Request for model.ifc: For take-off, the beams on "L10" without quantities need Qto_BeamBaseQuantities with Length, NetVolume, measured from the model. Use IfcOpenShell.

First a look at what the model holds.

```python
import ifcopenshell
import ifcopenshell.util.element
import ifcopenshell.util.unit

model = ifcopenshell.open("model.ifc")
print(model.schema)
for unit_type in ("LENGTHUNIT", "AREAUNIT", "VOLUMEUNIT"):
    print(unit_type, ifcopenshell.util.unit.calculate_unit_scale(model, unit_type))
storey = next(s for s in model.by_type("IfcBuildingStorey") if s.Name == "L10")
beams = [e for e in ifcopenshell.util.element.get_decomposition(storey) if e.is_a("IfcBeam")]
for e in sorted(beams, key=lambda e: e.id()):
    print(e.id(), e.is_a(), e.Name, list(ifcopenshell.util.element.get_psets(e, qtos_only=True)), sep=" | ")
```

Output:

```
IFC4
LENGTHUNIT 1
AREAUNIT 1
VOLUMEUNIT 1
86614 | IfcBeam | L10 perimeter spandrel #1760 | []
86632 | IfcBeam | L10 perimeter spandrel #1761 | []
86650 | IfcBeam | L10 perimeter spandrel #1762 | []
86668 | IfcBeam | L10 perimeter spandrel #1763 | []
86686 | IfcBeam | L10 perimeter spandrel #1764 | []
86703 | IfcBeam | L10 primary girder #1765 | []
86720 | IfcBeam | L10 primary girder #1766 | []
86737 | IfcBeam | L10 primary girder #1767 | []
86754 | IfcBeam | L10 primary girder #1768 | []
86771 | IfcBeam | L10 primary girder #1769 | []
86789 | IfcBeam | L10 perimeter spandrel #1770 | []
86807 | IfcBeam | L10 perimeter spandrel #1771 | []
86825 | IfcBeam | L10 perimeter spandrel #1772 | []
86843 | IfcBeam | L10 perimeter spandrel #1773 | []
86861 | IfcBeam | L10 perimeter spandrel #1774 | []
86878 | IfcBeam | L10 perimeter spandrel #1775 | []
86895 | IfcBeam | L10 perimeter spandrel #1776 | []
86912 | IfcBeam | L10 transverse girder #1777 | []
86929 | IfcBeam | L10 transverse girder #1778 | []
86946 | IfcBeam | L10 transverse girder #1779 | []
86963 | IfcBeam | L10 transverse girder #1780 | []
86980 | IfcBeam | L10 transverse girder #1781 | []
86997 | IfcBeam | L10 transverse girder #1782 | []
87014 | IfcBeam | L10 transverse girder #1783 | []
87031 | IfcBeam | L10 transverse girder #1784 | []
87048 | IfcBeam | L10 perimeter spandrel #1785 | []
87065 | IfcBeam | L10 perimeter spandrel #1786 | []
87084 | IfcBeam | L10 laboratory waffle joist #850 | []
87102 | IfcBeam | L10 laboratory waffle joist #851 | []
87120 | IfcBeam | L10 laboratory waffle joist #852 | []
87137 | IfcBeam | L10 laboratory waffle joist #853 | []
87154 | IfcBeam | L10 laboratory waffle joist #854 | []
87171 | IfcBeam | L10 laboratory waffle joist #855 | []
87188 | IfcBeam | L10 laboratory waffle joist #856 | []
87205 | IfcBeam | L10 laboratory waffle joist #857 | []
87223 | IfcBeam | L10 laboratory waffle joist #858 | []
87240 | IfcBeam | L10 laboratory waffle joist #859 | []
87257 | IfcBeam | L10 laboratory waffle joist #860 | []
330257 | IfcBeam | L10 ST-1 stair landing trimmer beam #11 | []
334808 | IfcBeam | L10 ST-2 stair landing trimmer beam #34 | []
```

```python
import ifcopenshell
import ifcopenshell.api.pset
import ifcopenshell.geom
import ifcopenshell.util.element
import ifcopenshell.util.shape
import ifcopenshell.util.unit

model = ifcopenshell.open("model.ifc")
unit_scale = ifcopenshell.util.unit.calculate_unit_scale(model)
volume_scale = ifcopenshell.util.unit.calculate_unit_scale(model, "VOLUMEUNIT")
settings = ifcopenshell.geom.settings()

storey = next(s for s in model.by_type("IfcBuildingStorey") if s.Name == "L10")
beams = [e for e in ifcopenshell.util.element.get_decomposition(storey) if e.is_a("IfcBeam")]

for e in sorted(beams, key=lambda e: e.id()):
    if ifcopenshell.util.element.get_psets(e, qtos_only=True, should_inherit=False):
        continue
    # Geometry comes back in metres, in the element's own axes.
    shape = ifcopenshell.geom.create_shape(settings, e)
    values = {
        "Length": ifcopenshell.util.shape.get_max_xyz(shape.geometry) / unit_scale,
        "NetVolume": ifcopenshell.util.shape.get_volume(shape.geometry) / volume_scale,
    }
    qto = ifcopenshell.api.pset.add_qto(model, product=e, name="Qto_BeamBaseQuantities")
    ifcopenshell.api.pset.edit_qto(model, qto=qto, properties=values)
    print(e.id(), {k: round(v, 3) for k, v in values.items()})

model.write("model_rev.ifc")
```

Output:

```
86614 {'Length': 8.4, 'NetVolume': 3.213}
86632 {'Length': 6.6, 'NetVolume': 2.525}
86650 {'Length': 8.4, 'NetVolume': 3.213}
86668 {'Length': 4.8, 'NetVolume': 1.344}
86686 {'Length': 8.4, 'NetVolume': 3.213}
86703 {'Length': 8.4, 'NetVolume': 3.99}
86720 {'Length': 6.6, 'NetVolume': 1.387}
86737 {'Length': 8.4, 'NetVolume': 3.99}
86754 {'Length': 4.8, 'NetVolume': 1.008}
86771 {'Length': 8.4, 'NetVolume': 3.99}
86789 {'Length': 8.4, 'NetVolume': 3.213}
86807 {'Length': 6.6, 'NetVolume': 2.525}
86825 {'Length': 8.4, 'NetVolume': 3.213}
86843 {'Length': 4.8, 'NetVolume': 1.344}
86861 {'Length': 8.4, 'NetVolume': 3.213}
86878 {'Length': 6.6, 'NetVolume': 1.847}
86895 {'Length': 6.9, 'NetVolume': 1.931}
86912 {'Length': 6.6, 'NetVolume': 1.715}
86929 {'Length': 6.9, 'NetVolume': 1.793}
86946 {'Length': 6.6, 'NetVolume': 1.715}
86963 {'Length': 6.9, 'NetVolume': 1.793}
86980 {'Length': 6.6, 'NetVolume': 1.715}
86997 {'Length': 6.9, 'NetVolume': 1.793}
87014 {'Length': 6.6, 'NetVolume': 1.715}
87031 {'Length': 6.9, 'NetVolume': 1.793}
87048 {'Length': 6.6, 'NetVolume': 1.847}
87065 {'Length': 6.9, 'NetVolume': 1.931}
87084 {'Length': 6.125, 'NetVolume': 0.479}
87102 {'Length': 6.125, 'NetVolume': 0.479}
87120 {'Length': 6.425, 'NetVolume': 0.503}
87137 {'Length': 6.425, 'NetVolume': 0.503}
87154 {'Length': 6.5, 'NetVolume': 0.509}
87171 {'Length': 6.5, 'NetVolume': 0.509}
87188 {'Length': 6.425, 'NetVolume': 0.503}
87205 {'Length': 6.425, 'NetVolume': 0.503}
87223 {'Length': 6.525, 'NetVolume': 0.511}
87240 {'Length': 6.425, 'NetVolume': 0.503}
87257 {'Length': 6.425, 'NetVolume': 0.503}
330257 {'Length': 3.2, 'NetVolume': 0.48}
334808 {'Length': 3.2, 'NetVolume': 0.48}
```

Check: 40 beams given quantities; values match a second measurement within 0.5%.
